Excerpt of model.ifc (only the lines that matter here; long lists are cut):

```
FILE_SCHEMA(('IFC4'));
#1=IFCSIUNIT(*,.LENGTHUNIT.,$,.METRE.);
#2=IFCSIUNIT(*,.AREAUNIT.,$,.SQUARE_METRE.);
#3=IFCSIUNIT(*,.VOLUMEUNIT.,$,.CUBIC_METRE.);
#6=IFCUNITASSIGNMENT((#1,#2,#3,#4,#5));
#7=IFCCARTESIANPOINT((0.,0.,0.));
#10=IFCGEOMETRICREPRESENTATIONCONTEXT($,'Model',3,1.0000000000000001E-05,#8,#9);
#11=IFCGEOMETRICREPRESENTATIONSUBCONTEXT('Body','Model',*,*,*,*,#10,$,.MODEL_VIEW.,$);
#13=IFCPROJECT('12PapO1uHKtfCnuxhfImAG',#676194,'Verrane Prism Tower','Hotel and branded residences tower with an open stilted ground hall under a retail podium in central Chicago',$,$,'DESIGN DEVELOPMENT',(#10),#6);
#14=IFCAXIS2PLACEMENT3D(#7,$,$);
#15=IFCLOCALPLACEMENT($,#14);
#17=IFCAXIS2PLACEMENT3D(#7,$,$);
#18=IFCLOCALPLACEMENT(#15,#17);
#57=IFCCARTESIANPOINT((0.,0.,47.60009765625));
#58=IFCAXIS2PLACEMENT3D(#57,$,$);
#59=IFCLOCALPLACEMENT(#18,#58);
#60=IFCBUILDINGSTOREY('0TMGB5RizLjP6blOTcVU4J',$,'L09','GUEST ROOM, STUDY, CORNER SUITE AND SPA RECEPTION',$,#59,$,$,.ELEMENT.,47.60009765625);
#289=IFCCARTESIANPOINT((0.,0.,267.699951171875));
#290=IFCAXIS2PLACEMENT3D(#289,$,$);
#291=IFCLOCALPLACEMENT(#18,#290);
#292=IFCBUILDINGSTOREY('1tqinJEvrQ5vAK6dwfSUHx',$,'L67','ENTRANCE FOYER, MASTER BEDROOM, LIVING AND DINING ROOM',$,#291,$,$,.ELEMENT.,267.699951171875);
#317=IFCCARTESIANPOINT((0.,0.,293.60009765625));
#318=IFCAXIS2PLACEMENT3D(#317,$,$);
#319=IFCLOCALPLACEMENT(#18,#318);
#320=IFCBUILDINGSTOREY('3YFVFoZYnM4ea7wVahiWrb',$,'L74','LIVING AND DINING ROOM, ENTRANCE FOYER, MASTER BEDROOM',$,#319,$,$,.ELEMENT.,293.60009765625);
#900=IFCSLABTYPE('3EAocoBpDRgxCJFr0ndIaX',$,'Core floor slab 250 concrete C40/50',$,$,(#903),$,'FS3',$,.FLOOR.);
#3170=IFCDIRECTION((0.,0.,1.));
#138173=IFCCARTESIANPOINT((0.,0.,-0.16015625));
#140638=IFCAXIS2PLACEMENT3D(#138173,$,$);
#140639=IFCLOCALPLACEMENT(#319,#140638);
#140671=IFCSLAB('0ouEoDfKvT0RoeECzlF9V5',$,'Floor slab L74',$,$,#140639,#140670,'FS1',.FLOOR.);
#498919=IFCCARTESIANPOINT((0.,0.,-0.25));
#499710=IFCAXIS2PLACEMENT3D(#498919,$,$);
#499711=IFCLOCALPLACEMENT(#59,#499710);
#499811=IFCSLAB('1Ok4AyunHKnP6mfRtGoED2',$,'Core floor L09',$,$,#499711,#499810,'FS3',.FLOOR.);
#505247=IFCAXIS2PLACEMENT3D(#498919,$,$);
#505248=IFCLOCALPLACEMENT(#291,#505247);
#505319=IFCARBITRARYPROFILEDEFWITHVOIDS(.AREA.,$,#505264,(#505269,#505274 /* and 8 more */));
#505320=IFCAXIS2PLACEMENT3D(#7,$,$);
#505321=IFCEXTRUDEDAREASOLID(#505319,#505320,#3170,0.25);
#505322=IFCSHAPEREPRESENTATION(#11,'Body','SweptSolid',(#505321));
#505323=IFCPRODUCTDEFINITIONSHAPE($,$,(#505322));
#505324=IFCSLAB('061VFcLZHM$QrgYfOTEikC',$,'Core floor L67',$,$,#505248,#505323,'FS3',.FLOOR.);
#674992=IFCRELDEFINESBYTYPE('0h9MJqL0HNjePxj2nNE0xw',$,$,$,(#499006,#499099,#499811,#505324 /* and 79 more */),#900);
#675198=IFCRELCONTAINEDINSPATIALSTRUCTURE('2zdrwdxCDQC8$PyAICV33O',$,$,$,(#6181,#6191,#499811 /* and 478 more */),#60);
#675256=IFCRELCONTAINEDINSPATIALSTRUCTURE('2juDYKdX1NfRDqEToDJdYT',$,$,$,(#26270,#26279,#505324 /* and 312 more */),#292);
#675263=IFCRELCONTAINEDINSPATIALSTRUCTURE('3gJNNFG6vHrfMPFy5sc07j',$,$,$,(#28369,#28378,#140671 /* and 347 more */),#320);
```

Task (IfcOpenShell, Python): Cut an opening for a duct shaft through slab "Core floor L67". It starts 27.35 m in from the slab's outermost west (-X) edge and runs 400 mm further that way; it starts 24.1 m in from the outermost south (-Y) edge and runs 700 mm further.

```python
import numpy as np
import ifcopenshell
import ifcopenshell.api.feature
import ifcopenshell.api.geometry
import ifcopenshell.api.root
import ifcopenshell.geom
import ifcopenshell.util.placement
import ifcopenshell.util.representation
import ifcopenshell.util.shape
import ifcopenshell.util.unit

model = ifcopenshell.open("model.ifc")
unit_scale = ifcopenshell.util.unit.calculate_unit_scale(model)
settings = ifcopenshell.geom.settings()


def volume(element):
    """Net volume in cubic metres, openings subtracted."""
    shape = ifcopenshell.geom.create_shape(settings, element)
    return ifcopenshell.util.shape.get_volume(shape.geometry)


slab = model.by_guid("061VFcLZHM$QrgYfOTEikC")
before = volume(slab)

# Extent in the slab's own axes, in metres. The edges named are its -X and -Y sides.
slab_shape = ifcopenshell.geom.create_shape(settings, slab)
vertices = ifcopenshell.util.shape.get_vertices(slab_shape.geometry)
x_min, y_min, bottom = vertices.min(axis=0)
top = vertices[:, 2].max()

opening = ifcopenshell.api.root.create_entity(model, ifc_class="IfcOpeningElement", name="Duct shaft opening", predefined_type="OPENING")
context = ifcopenshell.util.representation.get_context(model, "Model", "Body", "MODEL_VIEW")
width, depth = 0.4, 0.7
outline = [(0.0, 0.0), (width, 0.0), (width, depth), (0.0, depth), (0.0, 0.0)]
# Overshoot both faces by 50 mm so the cut is clean.
shape = ifcopenshell.api.geometry.add_slab_representation(
    model, context=context, depth=top - bottom + 0.1, polyline=outline
)
ifcopenshell.api.geometry.assign_representation(model, product=opening, representation=shape)

matrix = ifcopenshell.util.placement.get_local_placement(slab.ObjectPlacement)
matrix[:, 3] = matrix @ np.append(np.array([x_min + 27.35, y_min + 24.1, bottom - 0.05]) / unit_scale, 1.0)
ifcopenshell.api.geometry.edit_object_placement(model, product=opening, matrix=matrix, is_si=False)
ifcopenshell.api.feature.add_feature(model, feature=opening, element=slab)

after = volume(slab)

print(f"slab volume {before:.3f} -> {after:.3f} m3")

model.write("model-out.ifc")
```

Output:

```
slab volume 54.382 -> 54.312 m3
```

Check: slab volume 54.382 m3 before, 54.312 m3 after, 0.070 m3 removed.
